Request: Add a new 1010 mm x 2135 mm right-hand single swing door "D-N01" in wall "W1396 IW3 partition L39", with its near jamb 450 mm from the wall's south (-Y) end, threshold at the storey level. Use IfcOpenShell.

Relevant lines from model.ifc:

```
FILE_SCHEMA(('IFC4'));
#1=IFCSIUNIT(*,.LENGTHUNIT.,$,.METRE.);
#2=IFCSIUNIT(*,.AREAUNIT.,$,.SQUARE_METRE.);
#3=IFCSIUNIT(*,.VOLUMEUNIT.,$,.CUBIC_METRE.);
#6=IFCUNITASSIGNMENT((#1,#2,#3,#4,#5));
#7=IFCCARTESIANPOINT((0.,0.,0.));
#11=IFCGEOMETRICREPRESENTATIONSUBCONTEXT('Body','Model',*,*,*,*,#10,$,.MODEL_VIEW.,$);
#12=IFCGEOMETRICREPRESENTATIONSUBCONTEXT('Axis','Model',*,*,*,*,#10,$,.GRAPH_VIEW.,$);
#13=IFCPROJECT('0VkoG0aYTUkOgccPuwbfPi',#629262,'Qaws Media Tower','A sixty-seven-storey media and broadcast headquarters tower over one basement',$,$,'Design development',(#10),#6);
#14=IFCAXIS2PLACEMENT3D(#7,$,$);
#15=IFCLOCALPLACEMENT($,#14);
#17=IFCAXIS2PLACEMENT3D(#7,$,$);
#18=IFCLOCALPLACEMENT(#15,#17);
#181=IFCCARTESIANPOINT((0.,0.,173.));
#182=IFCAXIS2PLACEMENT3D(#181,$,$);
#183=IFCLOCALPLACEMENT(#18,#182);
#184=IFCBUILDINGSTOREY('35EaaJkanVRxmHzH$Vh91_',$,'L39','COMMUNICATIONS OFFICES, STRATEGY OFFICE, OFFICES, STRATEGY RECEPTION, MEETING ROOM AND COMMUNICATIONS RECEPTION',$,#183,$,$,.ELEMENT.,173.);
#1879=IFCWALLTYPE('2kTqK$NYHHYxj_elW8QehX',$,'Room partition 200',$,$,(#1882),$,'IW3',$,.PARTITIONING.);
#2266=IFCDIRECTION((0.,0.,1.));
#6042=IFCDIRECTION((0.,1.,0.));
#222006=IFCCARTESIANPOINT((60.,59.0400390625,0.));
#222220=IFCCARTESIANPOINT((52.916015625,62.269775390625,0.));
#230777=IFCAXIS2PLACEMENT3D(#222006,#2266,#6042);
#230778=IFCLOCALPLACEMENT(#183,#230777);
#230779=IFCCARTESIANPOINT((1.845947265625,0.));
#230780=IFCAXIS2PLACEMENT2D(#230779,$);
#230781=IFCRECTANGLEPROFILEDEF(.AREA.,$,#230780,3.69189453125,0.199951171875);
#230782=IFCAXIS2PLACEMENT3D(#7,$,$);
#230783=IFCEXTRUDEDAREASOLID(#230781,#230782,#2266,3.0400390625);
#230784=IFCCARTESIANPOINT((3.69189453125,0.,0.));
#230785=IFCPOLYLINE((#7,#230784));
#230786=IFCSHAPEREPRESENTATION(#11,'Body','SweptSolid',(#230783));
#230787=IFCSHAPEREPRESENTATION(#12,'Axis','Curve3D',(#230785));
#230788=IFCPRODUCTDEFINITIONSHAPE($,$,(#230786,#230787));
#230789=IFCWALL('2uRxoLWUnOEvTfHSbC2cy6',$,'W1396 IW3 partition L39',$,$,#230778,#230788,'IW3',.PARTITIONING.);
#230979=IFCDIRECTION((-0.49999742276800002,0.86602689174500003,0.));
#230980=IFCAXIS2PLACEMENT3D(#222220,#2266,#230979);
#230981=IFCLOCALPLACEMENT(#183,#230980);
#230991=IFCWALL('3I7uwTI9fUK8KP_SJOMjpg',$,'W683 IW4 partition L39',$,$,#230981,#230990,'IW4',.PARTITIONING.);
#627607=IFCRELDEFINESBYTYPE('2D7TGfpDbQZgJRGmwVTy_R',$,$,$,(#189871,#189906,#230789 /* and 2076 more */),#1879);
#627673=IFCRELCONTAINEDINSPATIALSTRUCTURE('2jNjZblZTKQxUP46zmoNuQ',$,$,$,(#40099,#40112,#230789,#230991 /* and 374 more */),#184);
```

```python
import numpy as np
import ifcopenshell
import ifcopenshell.api.feature
import ifcopenshell.api.geometry
import ifcopenshell.api.root
import ifcopenshell.api.spatial
import ifcopenshell.geom
import ifcopenshell.util.element
import ifcopenshell.util.placement
import ifcopenshell.util.representation
import ifcopenshell.util.shape
import ifcopenshell.util.unit

model = ifcopenshell.open("model.ifc")
unit_scale = ifcopenshell.util.unit.calculate_unit_scale(model)
settings = ifcopenshell.geom.settings()


def volume(element):
    """Net volume in cubic metres, openings subtracted."""
    shape = ifcopenshell.geom.create_shape(settings, element)
    return ifcopenshell.util.shape.get_volume(shape.geometry)


wall = model.by_id(230789)
storey = ifcopenshell.util.element.get_container(wall, ifc_class="IfcBuildingStorey")
context = ifcopenshell.util.representation.get_context(model, "Model", "Body", "MODEL_VIEW")
before = volume(wall)

width, height, from_end, sill = 1.01, 2.135, 0.45, 0.0  # metres

# The wall runs along its own X axis, and the end named is its -X end.
wall_shape = ifcopenshell.geom.create_shape(settings, wall)
x, y, z = ifcopenshell.util.shape.get_vertices(wall_shape.geometry).T
start = x.min() + from_end
face, thickness = float(y.min()), float(y.max() - y.min())
wall_matrix = ifcopenshell.util.placement.get_local_placement(wall.ObjectPlacement)
level = ifcopenshell.util.placement.get_local_placement(storey.ObjectPlacement)[2, 3]


def in_wall(x, y):
    """Placement at x, y metres in the wall's axes, at sill height."""
    matrix = wall_matrix.copy()
    matrix[:, 3] = wall_matrix @ np.array([x / unit_scale, y / unit_scale, 0.0, 1.0])
    matrix[2, 3] = level + sill / unit_scale
    return matrix


# Opening: a box that overshoots both wall faces by 50 mm.
opening = ifcopenshell.api.root.create_entity(model, ifc_class="IfcOpeningElement", predefined_type="OPENING")
box = ifcopenshell.api.geometry.add_wall_representation(
    model, context=context, length=width, height=height, thickness=thickness + 0.1
)
ifcopenshell.api.geometry.assign_representation(model, product=opening, representation=box)
ifcopenshell.api.geometry.edit_object_placement(model, product=opening, matrix=in_wall(start, face - 0.05), is_si=False)
ifcopenshell.api.feature.add_feature(model, feature=opening, element=wall)

door = ifcopenshell.api.root.create_entity(model, ifc_class="IfcDoor", name="D-N01", predefined_type="DOOR")
door.OverallWidth, door.OverallHeight = width / unit_scale, height / unit_scale
door.OperationType = "SINGLE_SWING_RIGHT"
body = ifcopenshell.api.geometry.add_door_representation(
    model,
    context=context,
    overall_width=door.OverallWidth,
    overall_height=door.OverallHeight,
    operation_type="SINGLE_SWING_RIGHT",
    lining_properties={"LiningDepth": thickness / unit_scale, "ThresholdDepth": thickness / unit_scale},
)
ifcopenshell.api.geometry.assign_representation(model, product=door, representation=body)
ifcopenshell.api.spatial.assign_container(model, products=[door], relating_structure=storey)
ifcopenshell.api.feature.add_filling(model, opening=opening, element=door)

# The lining spans the wall, so the door starts at the wall face.
ifcopenshell.api.geometry.edit_object_placement(model, product=door, matrix=in_wall(start, face), is_si=False)

after = volume(wall)

print(f"wall volume {before:.3f} -> {after:.3f} m3")

model.write("model_updated.ifc")
```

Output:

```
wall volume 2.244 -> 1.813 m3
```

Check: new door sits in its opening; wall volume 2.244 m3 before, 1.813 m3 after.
